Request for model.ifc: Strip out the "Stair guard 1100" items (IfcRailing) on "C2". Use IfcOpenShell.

First a look at what the model holds.

```python
import ifcopenshell
import ifcopenshell.util.element

model = ifcopenshell.open("model.ifc")
print(model.schema)
storey = next(s for s in model.by_type("IfcBuildingStorey") if s.Name == "C2")
railings = [e for e in ifcopenshell.util.element.get_decomposition(storey) if e.is_a("IfcRailing")]
seen = {}
for e in railings:
    element_type = ifcopenshell.util.element.get_type(e)
    name = element_type.Name if element_type not in (None, e) else None
    seen[name] = seen.get(name, 0) + 1
for name, count in sorted(seen.items(), key=str):
    print(count, "x", name)
```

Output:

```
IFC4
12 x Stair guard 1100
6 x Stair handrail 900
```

```python
import ifcopenshell
import ifcopenshell.api.root
import ifcopenshell.util.element

model = ifcopenshell.open("model.ifc")

storey = next(s for s in model.by_type("IfcBuildingStorey") if s.Name == "C2")
railings = [e for e in ifcopenshell.util.element.get_decomposition(storey) if e.is_a("IfcRailing")]
targets = [e for e in railings if (t := ifcopenshell.util.element.get_type(e)) not in (None, e) and t.Name == "Stair guard 1100"]

for e in targets:
    ifcopenshell.api.root.remove_product(model, product=e)
print(len(targets), "removed")

model.write("model_updated.ifc")
```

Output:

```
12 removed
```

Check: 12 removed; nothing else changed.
